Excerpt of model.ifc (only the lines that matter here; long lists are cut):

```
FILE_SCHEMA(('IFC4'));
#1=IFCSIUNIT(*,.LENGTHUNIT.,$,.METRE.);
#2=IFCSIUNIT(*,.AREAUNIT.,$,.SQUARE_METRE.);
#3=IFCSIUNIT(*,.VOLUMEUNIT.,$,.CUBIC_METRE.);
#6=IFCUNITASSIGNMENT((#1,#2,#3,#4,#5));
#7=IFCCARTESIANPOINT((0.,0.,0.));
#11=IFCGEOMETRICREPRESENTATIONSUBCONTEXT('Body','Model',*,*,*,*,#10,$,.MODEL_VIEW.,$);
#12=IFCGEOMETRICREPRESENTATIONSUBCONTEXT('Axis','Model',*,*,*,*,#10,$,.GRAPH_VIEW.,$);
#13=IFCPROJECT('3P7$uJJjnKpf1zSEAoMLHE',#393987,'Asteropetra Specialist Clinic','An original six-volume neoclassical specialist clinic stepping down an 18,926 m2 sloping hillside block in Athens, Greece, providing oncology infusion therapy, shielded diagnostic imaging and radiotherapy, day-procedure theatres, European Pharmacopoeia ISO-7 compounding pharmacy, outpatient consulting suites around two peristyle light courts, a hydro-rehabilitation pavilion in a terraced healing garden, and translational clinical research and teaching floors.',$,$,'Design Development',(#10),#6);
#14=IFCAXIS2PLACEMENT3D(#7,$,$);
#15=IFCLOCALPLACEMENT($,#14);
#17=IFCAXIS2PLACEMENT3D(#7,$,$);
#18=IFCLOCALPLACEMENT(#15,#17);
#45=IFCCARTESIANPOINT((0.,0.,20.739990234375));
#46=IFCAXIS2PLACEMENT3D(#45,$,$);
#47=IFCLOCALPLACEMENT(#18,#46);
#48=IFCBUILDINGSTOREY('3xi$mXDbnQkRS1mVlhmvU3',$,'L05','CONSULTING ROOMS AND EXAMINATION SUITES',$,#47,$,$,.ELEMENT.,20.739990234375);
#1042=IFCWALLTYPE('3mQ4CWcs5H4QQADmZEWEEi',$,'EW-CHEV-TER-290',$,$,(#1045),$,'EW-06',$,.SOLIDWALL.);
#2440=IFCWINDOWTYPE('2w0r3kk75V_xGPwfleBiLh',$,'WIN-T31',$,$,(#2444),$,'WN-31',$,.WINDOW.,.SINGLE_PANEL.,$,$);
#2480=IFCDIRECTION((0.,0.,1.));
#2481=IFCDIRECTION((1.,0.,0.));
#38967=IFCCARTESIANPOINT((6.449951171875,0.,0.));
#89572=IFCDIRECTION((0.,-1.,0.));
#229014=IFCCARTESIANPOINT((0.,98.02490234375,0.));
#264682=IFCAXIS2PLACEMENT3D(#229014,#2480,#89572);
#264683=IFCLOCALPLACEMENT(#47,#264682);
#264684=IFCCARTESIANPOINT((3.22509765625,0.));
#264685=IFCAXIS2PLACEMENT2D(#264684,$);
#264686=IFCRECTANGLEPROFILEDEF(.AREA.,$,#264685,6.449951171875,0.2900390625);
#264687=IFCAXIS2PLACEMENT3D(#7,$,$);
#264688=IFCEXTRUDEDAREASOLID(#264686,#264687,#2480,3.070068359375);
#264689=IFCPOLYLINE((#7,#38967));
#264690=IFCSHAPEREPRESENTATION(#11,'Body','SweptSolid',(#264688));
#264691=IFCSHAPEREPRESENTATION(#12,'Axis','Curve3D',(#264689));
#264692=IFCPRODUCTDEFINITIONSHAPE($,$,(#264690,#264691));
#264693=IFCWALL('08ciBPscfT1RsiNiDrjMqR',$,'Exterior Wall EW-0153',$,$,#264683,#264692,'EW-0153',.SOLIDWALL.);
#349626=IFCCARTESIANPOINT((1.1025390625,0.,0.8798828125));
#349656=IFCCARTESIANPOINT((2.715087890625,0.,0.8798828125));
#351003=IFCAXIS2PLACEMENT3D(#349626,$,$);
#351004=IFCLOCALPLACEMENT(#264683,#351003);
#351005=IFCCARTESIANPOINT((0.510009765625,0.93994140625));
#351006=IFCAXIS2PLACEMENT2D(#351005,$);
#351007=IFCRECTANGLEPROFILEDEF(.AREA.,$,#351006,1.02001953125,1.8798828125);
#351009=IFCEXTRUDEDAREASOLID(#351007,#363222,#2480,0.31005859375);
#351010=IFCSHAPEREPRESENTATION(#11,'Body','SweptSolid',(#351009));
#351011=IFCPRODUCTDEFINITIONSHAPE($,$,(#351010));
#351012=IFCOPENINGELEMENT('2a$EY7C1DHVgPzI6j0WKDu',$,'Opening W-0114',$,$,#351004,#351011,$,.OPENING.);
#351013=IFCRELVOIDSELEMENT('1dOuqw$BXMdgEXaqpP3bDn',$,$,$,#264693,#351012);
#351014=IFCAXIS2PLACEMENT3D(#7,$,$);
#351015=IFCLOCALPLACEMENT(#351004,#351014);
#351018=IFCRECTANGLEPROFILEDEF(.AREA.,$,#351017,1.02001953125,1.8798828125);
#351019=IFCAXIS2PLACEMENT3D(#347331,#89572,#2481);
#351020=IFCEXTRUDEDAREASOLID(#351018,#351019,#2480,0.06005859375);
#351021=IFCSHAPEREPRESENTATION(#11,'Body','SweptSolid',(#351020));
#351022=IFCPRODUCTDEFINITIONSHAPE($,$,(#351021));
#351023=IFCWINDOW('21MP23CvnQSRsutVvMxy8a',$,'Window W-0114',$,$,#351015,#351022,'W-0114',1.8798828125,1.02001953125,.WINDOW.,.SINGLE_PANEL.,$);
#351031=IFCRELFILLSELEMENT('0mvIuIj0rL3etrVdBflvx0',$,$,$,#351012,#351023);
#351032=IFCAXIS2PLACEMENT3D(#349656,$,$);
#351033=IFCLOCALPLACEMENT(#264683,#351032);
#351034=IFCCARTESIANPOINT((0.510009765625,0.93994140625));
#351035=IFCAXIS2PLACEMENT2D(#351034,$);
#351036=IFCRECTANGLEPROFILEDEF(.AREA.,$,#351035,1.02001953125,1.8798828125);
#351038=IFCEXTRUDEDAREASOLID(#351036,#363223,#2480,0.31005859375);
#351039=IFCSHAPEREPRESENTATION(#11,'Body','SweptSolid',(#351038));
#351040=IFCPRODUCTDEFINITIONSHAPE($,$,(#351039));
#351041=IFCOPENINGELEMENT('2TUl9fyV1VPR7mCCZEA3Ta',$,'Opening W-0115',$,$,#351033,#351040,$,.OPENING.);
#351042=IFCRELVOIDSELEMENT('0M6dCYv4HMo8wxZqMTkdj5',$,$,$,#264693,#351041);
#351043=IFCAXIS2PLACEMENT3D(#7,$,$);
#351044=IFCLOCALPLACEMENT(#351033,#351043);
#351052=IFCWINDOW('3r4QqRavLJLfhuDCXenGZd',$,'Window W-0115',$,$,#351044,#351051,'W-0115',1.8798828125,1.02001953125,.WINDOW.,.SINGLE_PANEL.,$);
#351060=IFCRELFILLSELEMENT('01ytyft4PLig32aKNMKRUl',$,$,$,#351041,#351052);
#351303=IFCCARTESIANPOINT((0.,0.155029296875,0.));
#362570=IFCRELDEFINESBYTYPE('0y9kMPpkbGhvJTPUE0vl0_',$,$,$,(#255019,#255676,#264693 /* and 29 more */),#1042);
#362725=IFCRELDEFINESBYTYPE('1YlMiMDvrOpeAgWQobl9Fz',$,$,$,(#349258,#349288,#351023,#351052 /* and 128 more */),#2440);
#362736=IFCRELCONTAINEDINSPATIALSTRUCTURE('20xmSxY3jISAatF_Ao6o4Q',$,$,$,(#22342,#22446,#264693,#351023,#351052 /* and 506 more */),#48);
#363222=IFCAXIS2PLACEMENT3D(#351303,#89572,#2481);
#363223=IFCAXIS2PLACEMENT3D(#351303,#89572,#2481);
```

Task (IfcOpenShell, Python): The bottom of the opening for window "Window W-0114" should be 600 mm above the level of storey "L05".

```python
import numpy as np
import ifcopenshell
import ifcopenshell.api.geometry
import ifcopenshell.geom
import ifcopenshell.util.element
import ifcopenshell.util.placement
import ifcopenshell.util.shape
import ifcopenshell.util.unit

model = ifcopenshell.open("model.ifc")
unit_scale = ifcopenshell.util.unit.calculate_unit_scale(model)

window = model.by_guid("21MP23CvnQSRsutVvMxy8a")
opening = window.FillsVoids[0].RelatingOpeningElement
storey = ifcopenshell.util.element.get_container(window, ifc_class="IfcBuildingStorey")
level = ifcopenshell.util.placement.get_local_placement(storey.ObjectPlacement)[2, 3]

# The opening's origin need not be at the sill, so measure its lowest point.
shape = ifcopenshell.geom.create_shape(ifcopenshell.geom.settings(), opening)
bottom = ifcopenshell.util.shape.get_shape_bottom_elevation(shape, shape.geometry) / unit_scale
dz = level + 0.6 - bottom

shift = np.array([0.0, 0.0, dz])
# The window is placed relative to its opening, so it follows when the opening moves.
matrix = ifcopenshell.util.placement.get_local_placement(opening.ObjectPlacement)
matrix[:3, 3] += shift
ifcopenshell.api.geometry.edit_object_placement(
    model, product=opening, matrix=matrix, is_si=False, should_transform_children=True
)

print(f"moved by {dz * unit_scale:+.3f} m")

model.write("model_updated.ifc")
```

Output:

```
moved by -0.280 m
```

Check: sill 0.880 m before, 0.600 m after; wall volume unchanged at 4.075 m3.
